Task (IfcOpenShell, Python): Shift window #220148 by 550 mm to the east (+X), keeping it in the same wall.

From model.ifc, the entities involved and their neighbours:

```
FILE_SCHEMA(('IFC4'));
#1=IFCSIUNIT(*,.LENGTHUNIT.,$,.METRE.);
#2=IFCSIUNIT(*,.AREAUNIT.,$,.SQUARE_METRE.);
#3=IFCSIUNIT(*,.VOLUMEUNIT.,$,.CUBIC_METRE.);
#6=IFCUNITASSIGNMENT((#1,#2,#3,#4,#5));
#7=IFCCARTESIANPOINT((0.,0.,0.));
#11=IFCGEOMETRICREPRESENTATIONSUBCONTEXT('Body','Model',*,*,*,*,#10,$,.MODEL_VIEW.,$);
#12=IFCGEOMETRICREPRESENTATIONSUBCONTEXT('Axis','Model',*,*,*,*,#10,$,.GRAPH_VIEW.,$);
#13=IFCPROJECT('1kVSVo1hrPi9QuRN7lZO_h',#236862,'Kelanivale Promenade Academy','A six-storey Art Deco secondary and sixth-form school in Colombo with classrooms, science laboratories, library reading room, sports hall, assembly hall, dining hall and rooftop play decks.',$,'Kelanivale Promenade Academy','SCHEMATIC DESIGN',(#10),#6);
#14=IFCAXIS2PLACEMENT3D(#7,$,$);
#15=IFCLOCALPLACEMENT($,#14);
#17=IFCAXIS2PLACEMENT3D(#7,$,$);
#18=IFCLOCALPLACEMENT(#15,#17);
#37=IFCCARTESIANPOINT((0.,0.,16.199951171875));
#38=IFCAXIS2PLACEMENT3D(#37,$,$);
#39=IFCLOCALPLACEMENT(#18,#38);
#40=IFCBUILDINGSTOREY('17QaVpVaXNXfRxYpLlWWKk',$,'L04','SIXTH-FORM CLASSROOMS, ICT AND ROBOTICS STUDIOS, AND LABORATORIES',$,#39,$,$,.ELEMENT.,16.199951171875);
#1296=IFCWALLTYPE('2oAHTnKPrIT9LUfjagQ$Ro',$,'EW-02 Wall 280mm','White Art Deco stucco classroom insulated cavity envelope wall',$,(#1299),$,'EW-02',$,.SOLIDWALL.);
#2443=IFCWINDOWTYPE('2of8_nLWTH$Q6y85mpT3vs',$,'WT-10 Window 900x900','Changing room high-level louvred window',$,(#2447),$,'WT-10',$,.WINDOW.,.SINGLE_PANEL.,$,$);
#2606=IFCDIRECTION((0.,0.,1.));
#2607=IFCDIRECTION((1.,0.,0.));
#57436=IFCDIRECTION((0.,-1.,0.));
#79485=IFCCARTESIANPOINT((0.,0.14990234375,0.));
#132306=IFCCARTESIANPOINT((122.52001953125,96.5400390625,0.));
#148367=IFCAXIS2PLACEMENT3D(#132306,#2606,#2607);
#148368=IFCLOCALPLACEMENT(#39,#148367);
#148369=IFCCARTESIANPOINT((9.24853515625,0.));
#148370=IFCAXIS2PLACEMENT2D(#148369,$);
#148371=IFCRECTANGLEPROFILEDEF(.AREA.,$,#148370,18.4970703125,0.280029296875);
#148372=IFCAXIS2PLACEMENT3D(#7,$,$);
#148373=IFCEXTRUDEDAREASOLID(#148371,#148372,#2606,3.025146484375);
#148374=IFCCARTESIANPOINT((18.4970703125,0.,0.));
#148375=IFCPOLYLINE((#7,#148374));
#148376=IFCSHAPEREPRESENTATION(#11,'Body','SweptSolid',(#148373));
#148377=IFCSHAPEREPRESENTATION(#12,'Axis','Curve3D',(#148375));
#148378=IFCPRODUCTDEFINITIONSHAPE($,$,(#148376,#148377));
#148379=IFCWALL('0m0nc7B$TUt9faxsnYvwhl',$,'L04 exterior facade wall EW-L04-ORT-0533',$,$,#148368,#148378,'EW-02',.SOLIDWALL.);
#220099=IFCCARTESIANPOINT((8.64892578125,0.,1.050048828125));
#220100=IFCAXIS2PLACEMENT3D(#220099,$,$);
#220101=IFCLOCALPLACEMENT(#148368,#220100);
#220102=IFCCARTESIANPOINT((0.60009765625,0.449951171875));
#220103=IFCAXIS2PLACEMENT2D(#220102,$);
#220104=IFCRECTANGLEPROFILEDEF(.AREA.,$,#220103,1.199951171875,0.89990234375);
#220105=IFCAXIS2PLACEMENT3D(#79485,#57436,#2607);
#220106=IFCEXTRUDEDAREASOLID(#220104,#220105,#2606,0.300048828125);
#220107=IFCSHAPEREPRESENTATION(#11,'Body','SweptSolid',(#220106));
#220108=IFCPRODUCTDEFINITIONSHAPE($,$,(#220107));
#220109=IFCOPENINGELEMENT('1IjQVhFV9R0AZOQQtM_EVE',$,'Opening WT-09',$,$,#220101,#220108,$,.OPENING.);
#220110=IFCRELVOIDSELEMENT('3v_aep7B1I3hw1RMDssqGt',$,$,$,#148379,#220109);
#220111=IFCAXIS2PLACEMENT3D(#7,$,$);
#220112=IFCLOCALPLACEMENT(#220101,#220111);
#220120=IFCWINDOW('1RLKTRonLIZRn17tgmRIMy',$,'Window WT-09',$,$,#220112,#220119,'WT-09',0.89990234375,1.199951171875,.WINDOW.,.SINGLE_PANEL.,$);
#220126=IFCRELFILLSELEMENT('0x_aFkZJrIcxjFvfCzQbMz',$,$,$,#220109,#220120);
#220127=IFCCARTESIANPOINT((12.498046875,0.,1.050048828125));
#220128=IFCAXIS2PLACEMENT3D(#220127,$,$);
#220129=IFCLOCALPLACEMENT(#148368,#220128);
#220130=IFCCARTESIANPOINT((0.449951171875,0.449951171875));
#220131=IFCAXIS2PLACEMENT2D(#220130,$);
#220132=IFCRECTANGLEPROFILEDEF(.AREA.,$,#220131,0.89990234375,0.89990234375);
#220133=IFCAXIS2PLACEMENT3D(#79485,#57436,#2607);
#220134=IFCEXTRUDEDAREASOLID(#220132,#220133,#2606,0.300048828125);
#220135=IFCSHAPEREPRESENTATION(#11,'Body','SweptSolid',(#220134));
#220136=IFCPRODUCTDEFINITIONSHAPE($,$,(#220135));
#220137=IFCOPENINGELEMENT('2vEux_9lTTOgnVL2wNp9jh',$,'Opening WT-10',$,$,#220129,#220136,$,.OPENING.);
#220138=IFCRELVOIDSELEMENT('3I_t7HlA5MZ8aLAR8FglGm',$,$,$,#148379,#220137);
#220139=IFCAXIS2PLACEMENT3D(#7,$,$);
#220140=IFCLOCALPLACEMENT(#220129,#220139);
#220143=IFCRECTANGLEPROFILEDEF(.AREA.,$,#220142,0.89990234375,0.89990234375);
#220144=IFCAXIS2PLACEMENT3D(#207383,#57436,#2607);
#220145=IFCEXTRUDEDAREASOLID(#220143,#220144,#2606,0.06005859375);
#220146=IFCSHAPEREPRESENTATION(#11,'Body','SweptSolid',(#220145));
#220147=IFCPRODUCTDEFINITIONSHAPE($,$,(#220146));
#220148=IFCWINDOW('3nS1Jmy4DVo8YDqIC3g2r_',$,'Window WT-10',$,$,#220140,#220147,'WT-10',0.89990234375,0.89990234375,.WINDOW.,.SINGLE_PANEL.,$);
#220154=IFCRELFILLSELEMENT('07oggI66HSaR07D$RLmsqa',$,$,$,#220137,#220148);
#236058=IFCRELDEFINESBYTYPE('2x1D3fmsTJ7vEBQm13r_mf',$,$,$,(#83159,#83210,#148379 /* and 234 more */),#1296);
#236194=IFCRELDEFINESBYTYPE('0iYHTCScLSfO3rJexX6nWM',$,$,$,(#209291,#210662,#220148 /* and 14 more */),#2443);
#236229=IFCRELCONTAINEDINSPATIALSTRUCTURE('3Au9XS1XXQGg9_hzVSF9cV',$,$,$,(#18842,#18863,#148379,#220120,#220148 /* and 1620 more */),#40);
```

```python
import ifcopenshell
import ifcopenshell.api.geometry
import ifcopenshell.util.placement

model = ifcopenshell.open("model.ifc")

window = model.by_id(220148)
opening = window.FillsVoids[0].RelatingOpeningElement
wall = opening.VoidsElements[0].RelatingBuildingElement

wall_matrix = ifcopenshell.util.placement.get_local_placement(wall.ObjectPlacement)
shift = wall_matrix[:3, 0] * 0.55
before = ifcopenshell.util.placement.get_local_placement(window.ObjectPlacement)[:3, 3].copy()

# The window is placed relative to its opening, so it follows when the opening moves.
matrix = ifcopenshell.util.placement.get_local_placement(opening.ObjectPlacement)
matrix[:3, 3] += shift
ifcopenshell.api.geometry.edit_object_placement(
    model, product=opening, matrix=matrix, is_si=False, should_transform_children=True
)

after = ifcopenshell.util.placement.get_local_placement(window.ObjectPlacement)[:3, 3]
print("window moved by", (after - before).round(3) + 0.0)

model.write("model_rev.ifc")
```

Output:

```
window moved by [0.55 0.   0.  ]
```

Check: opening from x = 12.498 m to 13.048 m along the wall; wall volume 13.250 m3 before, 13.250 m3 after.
